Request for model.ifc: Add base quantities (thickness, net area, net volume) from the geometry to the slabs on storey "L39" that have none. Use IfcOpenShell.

First a look at what the model holds.

```python
import ifcopenshell
import ifcopenshell.util.element
import ifcopenshell.util.unit

model = ifcopenshell.open("model.ifc")
print(model.schema)
for unit_type in ("LENGTHUNIT", "AREAUNIT", "VOLUMEUNIT"):
    print(unit_type, ifcopenshell.util.unit.calculate_unit_scale(model, unit_type))
storey = next(s for s in model.by_type("IfcBuildingStorey") if s.Name == "L39")
slabs = [e for e in ifcopenshell.util.element.get_decomposition(storey) if e.is_a("IfcSlab")]
for e in sorted(slabs, key=lambda e: e.id()):
    print(e.id(), e.is_a(), e.Name, list(ifcopenshell.util.element.get_psets(e, qtos_only=True)), sep=" | ")
```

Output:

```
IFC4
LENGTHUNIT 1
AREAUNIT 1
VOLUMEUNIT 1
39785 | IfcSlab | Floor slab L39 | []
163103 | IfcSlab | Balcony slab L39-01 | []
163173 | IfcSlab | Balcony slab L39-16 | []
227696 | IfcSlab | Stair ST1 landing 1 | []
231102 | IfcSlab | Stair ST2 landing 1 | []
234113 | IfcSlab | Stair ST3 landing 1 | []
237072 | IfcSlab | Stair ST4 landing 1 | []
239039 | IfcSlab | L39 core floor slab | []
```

```python
import ifcopenshell
import ifcopenshell.api.pset
import ifcopenshell.geom
import ifcopenshell.util.element
import ifcopenshell.util.shape
import ifcopenshell.util.unit

model = ifcopenshell.open("model.ifc")
unit_scale = ifcopenshell.util.unit.calculate_unit_scale(model)
area_scale = ifcopenshell.util.unit.calculate_unit_scale(model, "AREAUNIT")
volume_scale = ifcopenshell.util.unit.calculate_unit_scale(model, "VOLUMEUNIT")
settings = ifcopenshell.geom.settings()

storey = next(s for s in model.by_type("IfcBuildingStorey") if s.Name == "L39")
slabs = [e for e in ifcopenshell.util.element.get_decomposition(storey) if e.is_a("IfcSlab")]

for e in sorted(slabs, key=lambda e: e.id()):
    if ifcopenshell.util.element.get_psets(e, qtos_only=True, should_inherit=False):
        continue
    # Geometry comes back in metres, in the element's own axes.
    shape = ifcopenshell.geom.create_shape(settings, e)
    values = {
        "Width": ifcopenshell.util.shape.get_z(shape.geometry) / unit_scale,
        "NetArea": ifcopenshell.util.shape.get_footprint_area(shape.geometry) / area_scale,
        "NetVolume": ifcopenshell.util.shape.get_volume(shape.geometry) / volume_scale,
    }
    qto = ifcopenshell.api.pset.add_qto(model, product=e, name="Qto_SlabBaseQuantities")
    ifcopenshell.api.pset.edit_qto(model, qto=qto, properties=values)
    print(e.id(), {k: round(v, 3) for k, v in values.items()})

model.write("model_updated.ifc")
```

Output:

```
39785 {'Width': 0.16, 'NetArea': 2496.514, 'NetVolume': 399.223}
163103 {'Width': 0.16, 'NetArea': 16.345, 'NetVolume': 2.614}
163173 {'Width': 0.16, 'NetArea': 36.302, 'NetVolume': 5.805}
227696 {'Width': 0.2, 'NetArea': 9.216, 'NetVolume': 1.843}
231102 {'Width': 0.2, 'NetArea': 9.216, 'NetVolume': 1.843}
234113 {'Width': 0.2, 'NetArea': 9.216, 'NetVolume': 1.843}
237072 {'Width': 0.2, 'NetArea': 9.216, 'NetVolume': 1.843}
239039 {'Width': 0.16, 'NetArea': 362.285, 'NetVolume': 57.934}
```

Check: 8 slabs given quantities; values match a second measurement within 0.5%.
